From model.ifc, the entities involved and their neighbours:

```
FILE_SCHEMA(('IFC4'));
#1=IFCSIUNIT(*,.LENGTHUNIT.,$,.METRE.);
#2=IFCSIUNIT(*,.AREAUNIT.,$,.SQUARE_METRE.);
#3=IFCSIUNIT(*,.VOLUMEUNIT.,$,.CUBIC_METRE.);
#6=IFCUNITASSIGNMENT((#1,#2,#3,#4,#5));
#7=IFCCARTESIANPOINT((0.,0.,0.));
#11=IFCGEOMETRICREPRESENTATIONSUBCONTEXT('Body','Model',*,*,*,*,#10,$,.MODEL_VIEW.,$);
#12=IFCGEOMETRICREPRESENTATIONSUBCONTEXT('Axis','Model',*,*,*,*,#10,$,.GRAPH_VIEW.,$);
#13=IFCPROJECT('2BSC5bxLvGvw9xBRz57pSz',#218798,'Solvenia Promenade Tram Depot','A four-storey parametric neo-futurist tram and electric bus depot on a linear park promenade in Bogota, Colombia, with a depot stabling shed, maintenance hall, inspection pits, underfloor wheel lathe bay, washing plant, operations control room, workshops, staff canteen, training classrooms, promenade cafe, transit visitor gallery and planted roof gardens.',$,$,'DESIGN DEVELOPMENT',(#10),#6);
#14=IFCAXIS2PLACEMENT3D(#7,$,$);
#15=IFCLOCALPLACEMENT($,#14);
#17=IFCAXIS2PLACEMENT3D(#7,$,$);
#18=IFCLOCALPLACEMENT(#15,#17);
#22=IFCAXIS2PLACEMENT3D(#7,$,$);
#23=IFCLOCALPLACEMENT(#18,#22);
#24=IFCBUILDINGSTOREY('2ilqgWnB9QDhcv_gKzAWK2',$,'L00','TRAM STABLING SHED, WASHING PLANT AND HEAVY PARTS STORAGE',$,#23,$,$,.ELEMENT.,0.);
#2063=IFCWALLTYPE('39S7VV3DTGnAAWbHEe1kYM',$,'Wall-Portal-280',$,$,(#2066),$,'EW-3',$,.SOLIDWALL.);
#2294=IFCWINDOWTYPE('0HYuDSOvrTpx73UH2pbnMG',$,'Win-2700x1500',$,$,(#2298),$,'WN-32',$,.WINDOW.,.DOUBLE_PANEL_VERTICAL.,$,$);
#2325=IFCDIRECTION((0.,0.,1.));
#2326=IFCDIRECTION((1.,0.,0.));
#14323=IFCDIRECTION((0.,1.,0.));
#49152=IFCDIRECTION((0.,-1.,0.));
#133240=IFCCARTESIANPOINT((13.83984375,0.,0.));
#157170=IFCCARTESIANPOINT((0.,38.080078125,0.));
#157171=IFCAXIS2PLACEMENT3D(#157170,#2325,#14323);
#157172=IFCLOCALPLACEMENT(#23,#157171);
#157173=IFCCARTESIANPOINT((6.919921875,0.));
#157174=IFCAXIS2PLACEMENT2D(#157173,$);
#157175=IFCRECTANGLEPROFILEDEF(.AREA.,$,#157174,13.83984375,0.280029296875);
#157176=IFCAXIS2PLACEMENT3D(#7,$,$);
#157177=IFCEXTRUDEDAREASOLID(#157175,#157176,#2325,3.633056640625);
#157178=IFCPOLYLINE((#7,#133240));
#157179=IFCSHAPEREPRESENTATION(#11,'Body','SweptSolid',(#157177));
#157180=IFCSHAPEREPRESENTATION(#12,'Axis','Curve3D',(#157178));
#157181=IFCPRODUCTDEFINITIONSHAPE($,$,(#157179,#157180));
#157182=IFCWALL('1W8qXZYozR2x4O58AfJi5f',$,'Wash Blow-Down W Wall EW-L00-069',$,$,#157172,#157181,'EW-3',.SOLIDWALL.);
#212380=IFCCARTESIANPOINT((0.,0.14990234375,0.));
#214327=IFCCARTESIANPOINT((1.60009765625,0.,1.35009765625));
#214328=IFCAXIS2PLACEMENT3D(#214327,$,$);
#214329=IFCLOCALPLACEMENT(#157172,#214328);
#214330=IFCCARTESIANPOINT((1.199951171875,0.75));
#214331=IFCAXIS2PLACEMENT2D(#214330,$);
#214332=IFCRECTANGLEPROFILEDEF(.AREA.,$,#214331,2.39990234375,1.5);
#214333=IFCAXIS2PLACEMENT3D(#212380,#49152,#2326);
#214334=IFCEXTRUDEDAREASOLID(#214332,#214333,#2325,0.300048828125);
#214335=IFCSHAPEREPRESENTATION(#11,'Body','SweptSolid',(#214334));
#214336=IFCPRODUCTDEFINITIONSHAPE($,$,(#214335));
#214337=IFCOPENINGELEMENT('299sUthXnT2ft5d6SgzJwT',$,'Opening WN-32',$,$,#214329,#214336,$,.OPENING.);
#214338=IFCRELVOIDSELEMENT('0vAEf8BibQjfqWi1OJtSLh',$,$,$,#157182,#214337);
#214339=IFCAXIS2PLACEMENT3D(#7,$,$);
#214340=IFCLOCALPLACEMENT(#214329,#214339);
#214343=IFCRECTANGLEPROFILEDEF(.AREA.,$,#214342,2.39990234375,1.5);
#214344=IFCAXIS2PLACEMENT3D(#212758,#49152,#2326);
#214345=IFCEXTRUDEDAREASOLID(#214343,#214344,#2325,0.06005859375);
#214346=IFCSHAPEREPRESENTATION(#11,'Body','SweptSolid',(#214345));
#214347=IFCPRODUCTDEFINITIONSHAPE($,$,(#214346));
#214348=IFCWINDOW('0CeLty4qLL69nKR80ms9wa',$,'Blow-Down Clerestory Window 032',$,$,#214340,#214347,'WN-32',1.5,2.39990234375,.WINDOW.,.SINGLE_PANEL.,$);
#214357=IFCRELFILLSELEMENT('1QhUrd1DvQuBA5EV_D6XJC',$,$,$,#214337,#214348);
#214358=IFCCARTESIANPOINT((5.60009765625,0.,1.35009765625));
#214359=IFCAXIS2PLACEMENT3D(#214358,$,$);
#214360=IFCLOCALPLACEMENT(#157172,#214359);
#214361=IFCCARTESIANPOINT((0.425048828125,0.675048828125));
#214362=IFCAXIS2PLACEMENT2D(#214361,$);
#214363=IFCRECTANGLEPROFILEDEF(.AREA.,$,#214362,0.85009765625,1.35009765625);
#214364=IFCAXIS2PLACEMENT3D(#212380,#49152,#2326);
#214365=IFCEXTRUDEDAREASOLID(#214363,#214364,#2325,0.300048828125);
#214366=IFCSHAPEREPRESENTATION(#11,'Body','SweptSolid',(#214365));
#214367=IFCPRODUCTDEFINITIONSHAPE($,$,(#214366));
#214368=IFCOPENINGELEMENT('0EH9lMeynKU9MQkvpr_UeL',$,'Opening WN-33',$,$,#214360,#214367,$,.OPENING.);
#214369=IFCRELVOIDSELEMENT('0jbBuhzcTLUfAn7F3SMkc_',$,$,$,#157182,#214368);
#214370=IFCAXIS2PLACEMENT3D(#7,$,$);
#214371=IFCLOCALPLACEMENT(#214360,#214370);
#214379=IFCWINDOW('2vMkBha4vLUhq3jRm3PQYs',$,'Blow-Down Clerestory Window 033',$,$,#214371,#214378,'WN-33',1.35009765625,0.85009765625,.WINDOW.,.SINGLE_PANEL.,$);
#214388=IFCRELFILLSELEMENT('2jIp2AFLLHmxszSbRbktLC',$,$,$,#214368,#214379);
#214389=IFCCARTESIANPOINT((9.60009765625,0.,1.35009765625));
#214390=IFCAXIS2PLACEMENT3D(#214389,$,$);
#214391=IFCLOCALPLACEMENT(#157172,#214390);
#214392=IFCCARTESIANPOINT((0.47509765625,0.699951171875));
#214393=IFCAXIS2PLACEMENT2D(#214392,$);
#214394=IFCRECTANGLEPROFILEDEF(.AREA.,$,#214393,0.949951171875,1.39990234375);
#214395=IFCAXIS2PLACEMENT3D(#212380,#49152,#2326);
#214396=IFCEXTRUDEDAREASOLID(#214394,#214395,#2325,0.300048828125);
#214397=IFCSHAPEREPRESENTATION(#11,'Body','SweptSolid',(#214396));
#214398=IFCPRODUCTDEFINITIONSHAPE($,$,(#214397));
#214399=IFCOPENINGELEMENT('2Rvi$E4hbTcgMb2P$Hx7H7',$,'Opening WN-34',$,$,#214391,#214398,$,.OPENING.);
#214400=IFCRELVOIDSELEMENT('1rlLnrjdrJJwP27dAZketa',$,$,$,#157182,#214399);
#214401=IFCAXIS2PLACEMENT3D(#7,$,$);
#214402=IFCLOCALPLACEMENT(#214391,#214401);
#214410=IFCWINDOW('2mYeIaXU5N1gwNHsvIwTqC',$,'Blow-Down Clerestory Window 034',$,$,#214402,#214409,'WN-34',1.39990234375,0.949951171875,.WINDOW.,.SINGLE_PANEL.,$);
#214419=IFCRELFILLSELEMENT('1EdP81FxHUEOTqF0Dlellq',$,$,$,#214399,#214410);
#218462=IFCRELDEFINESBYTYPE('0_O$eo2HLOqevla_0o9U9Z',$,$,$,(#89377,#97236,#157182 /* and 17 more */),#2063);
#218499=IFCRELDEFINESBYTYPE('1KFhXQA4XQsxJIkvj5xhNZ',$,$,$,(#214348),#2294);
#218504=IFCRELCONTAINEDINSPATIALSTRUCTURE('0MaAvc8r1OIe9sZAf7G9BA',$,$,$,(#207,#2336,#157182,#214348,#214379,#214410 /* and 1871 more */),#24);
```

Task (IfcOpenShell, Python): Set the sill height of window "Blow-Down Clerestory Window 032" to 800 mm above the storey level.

```python
import numpy as np
import ifcopenshell
import ifcopenshell.api.geometry
import ifcopenshell.geom
import ifcopenshell.util.element
import ifcopenshell.util.placement
import ifcopenshell.util.shape
import ifcopenshell.util.unit

model = ifcopenshell.open("model.ifc")
unit_scale = ifcopenshell.util.unit.calculate_unit_scale(model)

window = model.by_guid("0CeLty4qLL69nKR80ms9wa")
opening = window.FillsVoids[0].RelatingOpeningElement
storey = ifcopenshell.util.element.get_container(window, ifc_class="IfcBuildingStorey")
level = ifcopenshell.util.placement.get_local_placement(storey.ObjectPlacement)[2, 3]

# The opening's origin need not be at the sill, so measure its lowest point.
shape = ifcopenshell.geom.create_shape(ifcopenshell.geom.settings(), opening)
bottom = ifcopenshell.util.shape.get_shape_bottom_elevation(shape, shape.geometry) / unit_scale
dz = level + 0.8 / unit_scale - bottom

shift = np.array([0.0, 0.0, dz])
# The window is placed relative to its opening, so it follows when the opening moves.
matrix = ifcopenshell.util.placement.get_local_placement(opening.ObjectPlacement)
matrix[:3, 3] += shift
ifcopenshell.api.geometry.edit_object_placement(
    model, product=opening, matrix=matrix, is_si=False, should_transform_children=True
)

print(f"moved by {dz * unit_scale:+.3f} m")

model.write("model-out.ifc")
```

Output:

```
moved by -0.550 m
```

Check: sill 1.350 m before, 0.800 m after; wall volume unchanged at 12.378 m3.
